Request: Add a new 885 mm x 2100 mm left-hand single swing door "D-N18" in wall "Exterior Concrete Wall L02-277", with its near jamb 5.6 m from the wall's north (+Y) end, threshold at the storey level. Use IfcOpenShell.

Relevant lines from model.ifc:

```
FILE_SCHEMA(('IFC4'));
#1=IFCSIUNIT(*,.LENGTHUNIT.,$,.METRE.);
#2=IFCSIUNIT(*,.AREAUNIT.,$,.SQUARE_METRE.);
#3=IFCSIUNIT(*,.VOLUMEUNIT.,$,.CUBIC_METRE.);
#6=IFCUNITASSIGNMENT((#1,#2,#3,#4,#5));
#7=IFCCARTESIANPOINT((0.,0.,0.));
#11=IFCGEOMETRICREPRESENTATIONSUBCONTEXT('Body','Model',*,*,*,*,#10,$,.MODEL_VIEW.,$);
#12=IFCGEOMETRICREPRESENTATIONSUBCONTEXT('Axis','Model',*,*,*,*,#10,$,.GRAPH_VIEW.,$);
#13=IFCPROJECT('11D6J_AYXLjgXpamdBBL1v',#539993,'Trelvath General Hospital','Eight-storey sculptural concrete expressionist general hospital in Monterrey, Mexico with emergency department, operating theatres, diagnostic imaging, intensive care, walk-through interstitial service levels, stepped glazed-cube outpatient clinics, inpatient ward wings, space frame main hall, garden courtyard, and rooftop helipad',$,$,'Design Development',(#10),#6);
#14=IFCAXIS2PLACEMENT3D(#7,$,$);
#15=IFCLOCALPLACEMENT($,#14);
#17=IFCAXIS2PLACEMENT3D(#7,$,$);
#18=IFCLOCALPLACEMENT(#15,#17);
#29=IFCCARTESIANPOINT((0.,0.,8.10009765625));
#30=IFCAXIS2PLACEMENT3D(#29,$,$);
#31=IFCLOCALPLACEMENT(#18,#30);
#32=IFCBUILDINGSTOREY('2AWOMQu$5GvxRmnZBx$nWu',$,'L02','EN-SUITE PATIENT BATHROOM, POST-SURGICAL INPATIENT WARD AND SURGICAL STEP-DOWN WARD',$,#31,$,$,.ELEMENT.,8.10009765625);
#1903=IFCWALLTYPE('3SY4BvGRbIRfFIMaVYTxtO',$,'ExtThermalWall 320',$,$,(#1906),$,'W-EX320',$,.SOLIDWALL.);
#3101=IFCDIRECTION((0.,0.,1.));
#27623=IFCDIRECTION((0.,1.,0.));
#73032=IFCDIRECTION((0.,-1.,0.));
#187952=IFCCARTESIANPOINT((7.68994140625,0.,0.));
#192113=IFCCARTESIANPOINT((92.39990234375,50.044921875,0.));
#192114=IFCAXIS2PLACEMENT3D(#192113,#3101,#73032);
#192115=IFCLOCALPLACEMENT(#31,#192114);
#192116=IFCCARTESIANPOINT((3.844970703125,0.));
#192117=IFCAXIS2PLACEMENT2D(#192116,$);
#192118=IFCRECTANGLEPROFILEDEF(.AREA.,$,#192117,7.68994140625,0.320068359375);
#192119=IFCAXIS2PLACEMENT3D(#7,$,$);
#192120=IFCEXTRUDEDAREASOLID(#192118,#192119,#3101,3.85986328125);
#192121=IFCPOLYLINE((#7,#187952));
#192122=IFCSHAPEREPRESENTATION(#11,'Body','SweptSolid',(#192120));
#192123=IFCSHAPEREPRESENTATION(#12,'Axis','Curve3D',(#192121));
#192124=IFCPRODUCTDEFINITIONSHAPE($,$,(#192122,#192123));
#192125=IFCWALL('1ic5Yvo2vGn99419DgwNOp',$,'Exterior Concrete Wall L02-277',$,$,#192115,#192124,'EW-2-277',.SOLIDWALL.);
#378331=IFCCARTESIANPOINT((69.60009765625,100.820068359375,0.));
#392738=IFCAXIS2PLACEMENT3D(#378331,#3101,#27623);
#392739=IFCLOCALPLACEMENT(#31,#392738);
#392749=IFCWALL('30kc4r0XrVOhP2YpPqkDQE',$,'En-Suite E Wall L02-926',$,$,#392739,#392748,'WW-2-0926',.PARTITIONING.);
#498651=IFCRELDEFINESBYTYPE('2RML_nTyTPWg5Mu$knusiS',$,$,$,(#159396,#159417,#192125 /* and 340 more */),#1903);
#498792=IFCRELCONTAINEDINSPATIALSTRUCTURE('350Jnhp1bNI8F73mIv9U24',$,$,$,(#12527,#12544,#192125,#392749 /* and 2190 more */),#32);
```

```python
import numpy as np
import ifcopenshell
import ifcopenshell.api.feature
import ifcopenshell.api.geometry
import ifcopenshell.api.root
import ifcopenshell.api.spatial
import ifcopenshell.geom
import ifcopenshell.util.element
import ifcopenshell.util.placement
import ifcopenshell.util.representation
import ifcopenshell.util.shape
import ifcopenshell.util.unit

model = ifcopenshell.open("model.ifc")
unit_scale = ifcopenshell.util.unit.calculate_unit_scale(model)
settings = ifcopenshell.geom.settings()


def volume(element):
    """Net volume in cubic metres, openings subtracted."""
    shape = ifcopenshell.geom.create_shape(settings, element)
    return ifcopenshell.util.shape.get_volume(shape.geometry)


wall = model.by_id(192125)
storey = ifcopenshell.util.element.get_container(wall, ifc_class="IfcBuildingStorey")
context = ifcopenshell.util.representation.get_context(model, "Model", "Body", "MODEL_VIEW")
before = volume(wall)

width, height, from_end, sill = 0.885, 2.1, 5.6, 0.0  # metres

# The wall runs along its own X axis, and the end named is its -X end.
wall_shape = ifcopenshell.geom.create_shape(settings, wall)
x, y, z = ifcopenshell.util.shape.get_vertices(wall_shape.geometry).T
start = x.min() + from_end
face, thickness = float(y.min()), float(y.max() - y.min())
wall_matrix = ifcopenshell.util.placement.get_local_placement(wall.ObjectPlacement)
level = ifcopenshell.util.placement.get_local_placement(storey.ObjectPlacement)[2, 3]


def in_wall(x, y):
    """Placement at x, y metres in the wall's axes, at sill height."""
    matrix = wall_matrix.copy()
    matrix[:, 3] = wall_matrix @ np.array([x / unit_scale, y / unit_scale, 0.0, 1.0])
    matrix[2, 3] = level + sill / unit_scale
    return matrix


# Opening: a box that overshoots both wall faces by 50 mm.
opening = ifcopenshell.api.root.create_entity(model, ifc_class="IfcOpeningElement", predefined_type="OPENING")
box = ifcopenshell.api.geometry.add_wall_representation(
    model, context=context, length=width, height=height, thickness=thickness + 0.1
)
ifcopenshell.api.geometry.assign_representation(model, product=opening, representation=box)
ifcopenshell.api.geometry.edit_object_placement(model, product=opening, matrix=in_wall(start, face - 0.05), is_si=False)
ifcopenshell.api.feature.add_feature(model, feature=opening, element=wall)

door = ifcopenshell.api.root.create_entity(model, ifc_class="IfcDoor", name="D-N18", predefined_type="DOOR")
door.OverallWidth, door.OverallHeight = width / unit_scale, height / unit_scale
door.OperationType = "SINGLE_SWING_LEFT"
body = ifcopenshell.api.geometry.add_door_representation(
    model,
    context=context,
    overall_width=door.OverallWidth,
    overall_height=door.OverallHeight,
    operation_type="SINGLE_SWING_LEFT",
    lining_properties={"LiningDepth": thickness / unit_scale, "ThresholdDepth": thickness / unit_scale},
)
ifcopenshell.api.geometry.assign_representation(model, product=door, representation=body)
ifcopenshell.api.spatial.assign_container(model, products=[door], relating_structure=storey)
ifcopenshell.api.feature.add_filling(model, opening=opening, element=door)

# The lining spans the wall, so the door starts at the wall face.
ifcopenshell.api.geometry.edit_object_placement(model, product=door, matrix=in_wall(start, face), is_si=False)

after = volume(wall)

print(f"wall volume {before:.3f} -> {after:.3f} m3")

model.write("model_v2.ifc")
```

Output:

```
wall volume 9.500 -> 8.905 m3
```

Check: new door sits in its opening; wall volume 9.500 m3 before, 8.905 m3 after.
